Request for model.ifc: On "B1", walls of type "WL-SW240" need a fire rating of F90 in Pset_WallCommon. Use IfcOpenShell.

First a look at what the model holds.

```python
import ifcopenshell
import ifcopenshell.util.element

model = ifcopenshell.open("model.ifc")
print(model.schema)
storey = next(s for s in model.by_type("IfcBuildingStorey") if s.Name == "B1")
walls = [e for e in ifcopenshell.util.element.get_decomposition(storey) if e.is_a("IfcWall")]
seen = {}
for e in walls:
    element_type = ifcopenshell.util.element.get_type(e)
    key = (element_type.Name if element_type != e and element_type else None, ifcopenshell.util.element.get_pset(e, "Pset_WallCommon", "FireRating"))
    seen[key] = seen.get(key, 0) + 1
for (name, value), count in sorted(seen.items(), key=str):
    print(count, "x", name, "|", value)
```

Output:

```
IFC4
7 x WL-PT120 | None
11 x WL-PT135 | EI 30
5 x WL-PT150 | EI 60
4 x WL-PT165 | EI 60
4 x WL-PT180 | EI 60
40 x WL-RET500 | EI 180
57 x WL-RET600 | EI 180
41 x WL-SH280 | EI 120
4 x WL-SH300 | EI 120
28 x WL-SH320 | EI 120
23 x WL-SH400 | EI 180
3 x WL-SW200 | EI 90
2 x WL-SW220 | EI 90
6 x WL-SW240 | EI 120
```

```python
import ifcopenshell
import ifcopenshell.api.pset
import ifcopenshell.util.element

model = ifcopenshell.open("model.ifc")

storey = next(s for s in model.by_type("IfcBuildingStorey") if s.Name == "B1")
walls = [e for e in ifcopenshell.util.element.get_decomposition(storey) if e.is_a("IfcWall")]

count = 0
for e in walls:
    element_type = ifcopenshell.util.element.get_type(e)
    if element_type in (None, e) or element_type.Name != "WL-SW240":
        continue
    # add_pset returns the element's existing set when there is one.
    pset = ifcopenshell.api.pset.add_pset(model, product=e, name="Pset_WallCommon")
    ifcopenshell.api.pset.edit_pset(model, pset=pset, properties={"FireRating": "F90"})
    count += 1

print(count, "walls updated")

model.write("model_v2.ifc")
```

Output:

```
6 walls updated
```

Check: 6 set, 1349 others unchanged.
